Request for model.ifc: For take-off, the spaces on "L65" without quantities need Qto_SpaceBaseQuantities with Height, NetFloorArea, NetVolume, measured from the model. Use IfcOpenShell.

First a look at what the model holds.

```python
import ifcopenshell
import ifcopenshell.util.element
import ifcopenshell.util.unit

model = ifcopenshell.open("model.ifc")
print(model.schema)
for unit_type in ("LENGTHUNIT", "AREAUNIT", "VOLUMEUNIT"):
    print(unit_type, ifcopenshell.util.unit.calculate_unit_scale(model, unit_type))
storey = next(s for s in model.by_type("IfcBuildingStorey") if s.Name == "L65")
spaces = [e for e in ifcopenshell.util.element.get_decomposition(storey) if e.is_a("IfcSpace")]
for e in sorted(spaces, key=lambda e: e.id()):
    print(e.id(), e.is_a(), e.Name, list(ifcopenshell.util.element.get_psets(e, qtos_only=True)), sep=" | ")
```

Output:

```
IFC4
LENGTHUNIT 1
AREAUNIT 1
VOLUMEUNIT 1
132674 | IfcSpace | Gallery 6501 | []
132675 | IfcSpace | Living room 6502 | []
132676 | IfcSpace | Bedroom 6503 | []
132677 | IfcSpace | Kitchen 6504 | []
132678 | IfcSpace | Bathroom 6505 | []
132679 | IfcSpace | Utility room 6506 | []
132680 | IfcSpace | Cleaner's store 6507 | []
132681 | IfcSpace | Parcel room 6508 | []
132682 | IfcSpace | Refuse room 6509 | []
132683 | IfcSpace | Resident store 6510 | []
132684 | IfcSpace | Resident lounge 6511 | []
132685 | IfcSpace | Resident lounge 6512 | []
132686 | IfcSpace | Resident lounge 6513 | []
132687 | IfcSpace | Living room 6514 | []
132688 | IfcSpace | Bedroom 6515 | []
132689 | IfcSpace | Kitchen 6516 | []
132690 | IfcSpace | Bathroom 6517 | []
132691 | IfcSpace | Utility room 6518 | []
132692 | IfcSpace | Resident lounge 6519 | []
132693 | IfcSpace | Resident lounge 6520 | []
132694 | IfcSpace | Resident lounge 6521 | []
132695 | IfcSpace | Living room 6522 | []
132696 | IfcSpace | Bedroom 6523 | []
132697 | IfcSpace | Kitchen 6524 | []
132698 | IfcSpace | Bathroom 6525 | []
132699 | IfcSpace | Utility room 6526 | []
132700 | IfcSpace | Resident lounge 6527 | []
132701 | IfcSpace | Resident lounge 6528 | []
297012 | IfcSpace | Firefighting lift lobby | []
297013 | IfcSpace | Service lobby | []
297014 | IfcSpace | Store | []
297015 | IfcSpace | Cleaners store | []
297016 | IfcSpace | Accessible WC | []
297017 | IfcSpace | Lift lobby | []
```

```python
import ifcopenshell
import ifcopenshell.api.pset
import ifcopenshell.geom
import ifcopenshell.util.element
import ifcopenshell.util.shape
import ifcopenshell.util.unit

model = ifcopenshell.open("model.ifc")
unit_scale = ifcopenshell.util.unit.calculate_unit_scale(model)
area_scale = ifcopenshell.util.unit.calculate_unit_scale(model, "AREAUNIT")
volume_scale = ifcopenshell.util.unit.calculate_unit_scale(model, "VOLUMEUNIT")
settings = ifcopenshell.geom.settings()

storey = next(s for s in model.by_type("IfcBuildingStorey") if s.Name == "L65")
spaces = [e for e in ifcopenshell.util.element.get_decomposition(storey) if e.is_a("IfcSpace")]

for e in sorted(spaces, key=lambda e: e.id()):
    if ifcopenshell.util.element.get_psets(e, qtos_only=True, should_inherit=False):
        continue
    # Geometry comes back in metres, in the element's own axes.
    shape = ifcopenshell.geom.create_shape(settings, e)
    values = {
        "Height": ifcopenshell.util.shape.get_z(shape.geometry) / unit_scale,
        "NetFloorArea": ifcopenshell.util.shape.get_footprint_area(shape.geometry) / area_scale,
        "NetVolume": ifcopenshell.util.shape.get_volume(shape.geometry) / volume_scale,
    }
    qto = ifcopenshell.api.pset.add_qto(model, product=e, name="Qto_SpaceBaseQuantities")
    ifcopenshell.api.pset.edit_qto(model, qto=qto, properties=values)
    print(e.id(), {k: round(v, 3) for k, v in values.items()})

model.write("model-out.ifc")
```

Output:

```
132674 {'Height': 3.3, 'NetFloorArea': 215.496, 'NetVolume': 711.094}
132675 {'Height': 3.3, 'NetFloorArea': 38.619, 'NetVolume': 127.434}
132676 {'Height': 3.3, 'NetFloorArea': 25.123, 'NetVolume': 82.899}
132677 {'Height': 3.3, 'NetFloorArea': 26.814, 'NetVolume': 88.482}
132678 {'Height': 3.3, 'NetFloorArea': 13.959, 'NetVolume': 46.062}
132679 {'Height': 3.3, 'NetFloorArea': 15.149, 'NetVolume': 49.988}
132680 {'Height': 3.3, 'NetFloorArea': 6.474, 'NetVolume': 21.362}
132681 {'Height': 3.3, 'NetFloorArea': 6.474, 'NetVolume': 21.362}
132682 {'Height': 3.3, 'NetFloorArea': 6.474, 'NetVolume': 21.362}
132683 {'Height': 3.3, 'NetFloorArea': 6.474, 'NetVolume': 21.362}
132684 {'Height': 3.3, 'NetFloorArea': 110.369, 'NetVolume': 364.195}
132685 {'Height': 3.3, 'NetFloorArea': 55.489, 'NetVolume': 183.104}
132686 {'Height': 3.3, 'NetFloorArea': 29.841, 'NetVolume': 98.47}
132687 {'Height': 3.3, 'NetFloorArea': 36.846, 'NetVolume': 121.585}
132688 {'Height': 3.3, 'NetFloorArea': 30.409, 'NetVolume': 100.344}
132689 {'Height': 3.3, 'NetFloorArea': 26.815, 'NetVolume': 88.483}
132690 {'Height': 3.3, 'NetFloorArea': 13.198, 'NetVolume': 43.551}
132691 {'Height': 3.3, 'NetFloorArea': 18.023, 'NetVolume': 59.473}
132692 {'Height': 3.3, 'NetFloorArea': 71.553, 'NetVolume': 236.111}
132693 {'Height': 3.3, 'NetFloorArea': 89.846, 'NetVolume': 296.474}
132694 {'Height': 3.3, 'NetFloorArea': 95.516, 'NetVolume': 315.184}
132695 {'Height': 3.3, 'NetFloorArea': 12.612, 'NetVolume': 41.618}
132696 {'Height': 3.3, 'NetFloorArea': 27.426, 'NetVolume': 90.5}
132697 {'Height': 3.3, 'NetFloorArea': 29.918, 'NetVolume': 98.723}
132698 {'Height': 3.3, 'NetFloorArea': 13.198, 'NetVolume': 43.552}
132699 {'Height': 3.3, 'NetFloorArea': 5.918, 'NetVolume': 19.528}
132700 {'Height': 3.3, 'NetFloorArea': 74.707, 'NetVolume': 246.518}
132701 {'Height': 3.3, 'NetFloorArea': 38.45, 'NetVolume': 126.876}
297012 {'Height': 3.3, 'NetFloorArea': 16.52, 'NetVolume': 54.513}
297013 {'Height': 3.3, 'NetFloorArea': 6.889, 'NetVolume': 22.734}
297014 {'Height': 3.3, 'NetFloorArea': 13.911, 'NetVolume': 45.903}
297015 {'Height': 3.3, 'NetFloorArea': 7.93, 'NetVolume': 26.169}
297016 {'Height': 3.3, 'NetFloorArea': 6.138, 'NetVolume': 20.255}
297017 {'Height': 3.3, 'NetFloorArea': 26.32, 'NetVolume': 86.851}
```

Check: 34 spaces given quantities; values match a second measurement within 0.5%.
